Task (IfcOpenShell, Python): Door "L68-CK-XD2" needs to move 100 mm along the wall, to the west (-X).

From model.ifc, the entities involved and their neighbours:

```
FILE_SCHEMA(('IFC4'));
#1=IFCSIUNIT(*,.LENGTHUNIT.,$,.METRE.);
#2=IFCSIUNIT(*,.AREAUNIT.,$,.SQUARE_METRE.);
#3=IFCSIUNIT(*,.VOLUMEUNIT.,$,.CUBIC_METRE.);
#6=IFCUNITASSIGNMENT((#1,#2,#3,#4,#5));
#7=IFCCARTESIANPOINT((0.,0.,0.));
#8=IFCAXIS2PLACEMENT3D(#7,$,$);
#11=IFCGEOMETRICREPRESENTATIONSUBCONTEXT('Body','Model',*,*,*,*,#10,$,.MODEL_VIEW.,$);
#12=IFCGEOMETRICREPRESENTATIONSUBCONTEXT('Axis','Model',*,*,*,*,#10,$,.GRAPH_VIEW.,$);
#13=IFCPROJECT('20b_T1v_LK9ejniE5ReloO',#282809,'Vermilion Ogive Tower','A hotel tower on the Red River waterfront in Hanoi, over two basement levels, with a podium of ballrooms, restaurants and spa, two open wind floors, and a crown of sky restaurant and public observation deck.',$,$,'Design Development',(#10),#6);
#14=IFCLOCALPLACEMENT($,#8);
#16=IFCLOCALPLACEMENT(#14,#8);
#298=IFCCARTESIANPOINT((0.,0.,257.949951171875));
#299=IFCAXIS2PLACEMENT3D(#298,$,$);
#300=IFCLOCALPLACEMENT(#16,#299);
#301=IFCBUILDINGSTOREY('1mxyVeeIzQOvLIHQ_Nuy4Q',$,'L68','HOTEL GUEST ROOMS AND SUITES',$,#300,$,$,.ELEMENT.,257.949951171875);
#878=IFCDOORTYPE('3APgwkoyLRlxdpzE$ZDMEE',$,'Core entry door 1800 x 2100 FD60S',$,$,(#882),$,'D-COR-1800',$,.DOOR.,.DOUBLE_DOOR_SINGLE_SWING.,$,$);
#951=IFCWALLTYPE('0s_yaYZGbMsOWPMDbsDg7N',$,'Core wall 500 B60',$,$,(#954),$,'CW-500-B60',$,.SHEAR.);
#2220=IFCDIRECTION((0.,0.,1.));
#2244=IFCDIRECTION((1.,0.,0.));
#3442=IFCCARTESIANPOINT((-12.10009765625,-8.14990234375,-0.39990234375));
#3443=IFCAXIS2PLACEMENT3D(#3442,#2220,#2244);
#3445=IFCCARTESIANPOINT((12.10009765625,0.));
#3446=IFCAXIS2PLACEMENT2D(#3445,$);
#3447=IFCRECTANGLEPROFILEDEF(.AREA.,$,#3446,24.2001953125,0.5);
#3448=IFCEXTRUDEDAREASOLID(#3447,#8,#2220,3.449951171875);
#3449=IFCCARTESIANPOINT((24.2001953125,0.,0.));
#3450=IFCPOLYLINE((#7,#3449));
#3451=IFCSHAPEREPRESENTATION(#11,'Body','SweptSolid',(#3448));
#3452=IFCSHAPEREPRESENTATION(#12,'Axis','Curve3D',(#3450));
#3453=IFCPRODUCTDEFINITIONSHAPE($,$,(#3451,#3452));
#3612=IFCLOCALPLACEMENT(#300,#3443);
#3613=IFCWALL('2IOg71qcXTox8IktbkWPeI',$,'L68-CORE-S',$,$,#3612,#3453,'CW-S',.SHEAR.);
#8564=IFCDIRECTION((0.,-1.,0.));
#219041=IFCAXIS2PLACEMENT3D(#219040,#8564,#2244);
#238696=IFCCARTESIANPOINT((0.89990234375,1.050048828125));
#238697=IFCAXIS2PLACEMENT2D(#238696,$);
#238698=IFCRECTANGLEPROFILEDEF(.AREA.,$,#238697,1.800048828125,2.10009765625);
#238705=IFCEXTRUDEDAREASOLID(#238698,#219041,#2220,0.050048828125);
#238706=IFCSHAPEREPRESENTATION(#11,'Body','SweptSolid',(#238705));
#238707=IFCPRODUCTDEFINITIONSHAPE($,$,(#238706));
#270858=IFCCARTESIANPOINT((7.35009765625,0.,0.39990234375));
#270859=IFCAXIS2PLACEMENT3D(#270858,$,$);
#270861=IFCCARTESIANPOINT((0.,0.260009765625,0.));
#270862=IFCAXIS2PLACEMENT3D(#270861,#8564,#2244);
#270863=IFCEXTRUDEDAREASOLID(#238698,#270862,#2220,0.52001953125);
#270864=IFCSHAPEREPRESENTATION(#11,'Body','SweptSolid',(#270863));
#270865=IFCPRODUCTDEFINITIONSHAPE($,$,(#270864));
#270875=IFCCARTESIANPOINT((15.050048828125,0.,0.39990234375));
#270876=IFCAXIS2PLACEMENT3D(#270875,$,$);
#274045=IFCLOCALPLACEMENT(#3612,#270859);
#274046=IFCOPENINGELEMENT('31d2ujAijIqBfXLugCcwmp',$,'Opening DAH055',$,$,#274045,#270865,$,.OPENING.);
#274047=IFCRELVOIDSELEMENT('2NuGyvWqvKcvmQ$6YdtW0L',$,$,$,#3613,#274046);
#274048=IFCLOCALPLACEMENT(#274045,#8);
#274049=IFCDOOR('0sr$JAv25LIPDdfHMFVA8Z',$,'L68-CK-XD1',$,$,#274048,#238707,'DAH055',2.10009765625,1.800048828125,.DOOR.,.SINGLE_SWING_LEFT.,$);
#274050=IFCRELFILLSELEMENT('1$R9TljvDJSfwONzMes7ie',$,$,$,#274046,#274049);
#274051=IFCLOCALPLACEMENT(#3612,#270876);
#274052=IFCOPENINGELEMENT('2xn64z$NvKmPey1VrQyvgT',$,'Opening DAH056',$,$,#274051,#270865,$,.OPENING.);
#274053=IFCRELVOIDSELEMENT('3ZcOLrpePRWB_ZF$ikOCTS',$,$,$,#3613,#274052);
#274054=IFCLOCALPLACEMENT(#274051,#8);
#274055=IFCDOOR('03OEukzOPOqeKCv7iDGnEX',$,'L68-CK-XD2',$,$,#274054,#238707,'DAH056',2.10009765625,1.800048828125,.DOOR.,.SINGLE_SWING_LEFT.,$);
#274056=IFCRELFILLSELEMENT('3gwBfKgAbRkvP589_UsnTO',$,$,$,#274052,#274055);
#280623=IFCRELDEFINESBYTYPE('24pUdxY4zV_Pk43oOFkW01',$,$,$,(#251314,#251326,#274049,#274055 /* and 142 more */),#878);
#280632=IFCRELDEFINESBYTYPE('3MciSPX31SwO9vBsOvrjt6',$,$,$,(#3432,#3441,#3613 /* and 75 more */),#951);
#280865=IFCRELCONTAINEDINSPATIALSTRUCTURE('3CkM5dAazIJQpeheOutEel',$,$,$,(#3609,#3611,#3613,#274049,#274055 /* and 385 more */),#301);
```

```python
import ifcopenshell
import ifcopenshell.api.geometry
import ifcopenshell.util.placement

model = ifcopenshell.open("model.ifc")

door = model.by_guid("03OEukzOPOqeKCv7iDGnEX")
opening = door.FillsVoids[0].RelatingOpeningElement
wall = opening.VoidsElements[0].RelatingBuildingElement

wall_matrix = ifcopenshell.util.placement.get_local_placement(wall.ObjectPlacement)
shift = wall_matrix[:3, 0] * -0.1
before = ifcopenshell.util.placement.get_local_placement(door.ObjectPlacement)[:3, 3].copy()

# The door is placed relative to its opening, so it follows when the opening moves.
matrix = ifcopenshell.util.placement.get_local_placement(opening.ObjectPlacement)
matrix[:3, 3] += shift
ifcopenshell.api.geometry.edit_object_placement(
    model, product=opening, matrix=matrix, is_si=False, should_transform_children=True
)

after = ifcopenshell.util.placement.get_local_placement(door.ObjectPlacement)[:3, 3]
print("door moved by", (after - before).round(3) + 0.0)

model.write("model_rev.ifc")
```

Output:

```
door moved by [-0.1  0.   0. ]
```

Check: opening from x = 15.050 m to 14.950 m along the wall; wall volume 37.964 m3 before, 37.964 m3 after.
